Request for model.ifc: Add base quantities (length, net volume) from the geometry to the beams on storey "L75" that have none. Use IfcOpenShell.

First a look at what the model holds.

```python
import ifcopenshell
import ifcopenshell.util.element
import ifcopenshell.util.unit

model = ifcopenshell.open("model.ifc")
print(model.schema)
for unit_type in ("LENGTHUNIT", "AREAUNIT", "VOLUMEUNIT"):
    print(unit_type, ifcopenshell.util.unit.calculate_unit_scale(model, unit_type))
storey = next(s for s in model.by_type("IfcBuildingStorey") if s.Name == "L75")
beams = [e for e in ifcopenshell.util.element.get_decomposition(storey) if e.is_a("IfcBeam")]
for e in sorted(beams, key=lambda e: e.id()):
    print(e.id(), e.is_a(), e.Name, list(ifcopenshell.util.element.get_psets(e, qtos_only=True)), sep=" | ")
```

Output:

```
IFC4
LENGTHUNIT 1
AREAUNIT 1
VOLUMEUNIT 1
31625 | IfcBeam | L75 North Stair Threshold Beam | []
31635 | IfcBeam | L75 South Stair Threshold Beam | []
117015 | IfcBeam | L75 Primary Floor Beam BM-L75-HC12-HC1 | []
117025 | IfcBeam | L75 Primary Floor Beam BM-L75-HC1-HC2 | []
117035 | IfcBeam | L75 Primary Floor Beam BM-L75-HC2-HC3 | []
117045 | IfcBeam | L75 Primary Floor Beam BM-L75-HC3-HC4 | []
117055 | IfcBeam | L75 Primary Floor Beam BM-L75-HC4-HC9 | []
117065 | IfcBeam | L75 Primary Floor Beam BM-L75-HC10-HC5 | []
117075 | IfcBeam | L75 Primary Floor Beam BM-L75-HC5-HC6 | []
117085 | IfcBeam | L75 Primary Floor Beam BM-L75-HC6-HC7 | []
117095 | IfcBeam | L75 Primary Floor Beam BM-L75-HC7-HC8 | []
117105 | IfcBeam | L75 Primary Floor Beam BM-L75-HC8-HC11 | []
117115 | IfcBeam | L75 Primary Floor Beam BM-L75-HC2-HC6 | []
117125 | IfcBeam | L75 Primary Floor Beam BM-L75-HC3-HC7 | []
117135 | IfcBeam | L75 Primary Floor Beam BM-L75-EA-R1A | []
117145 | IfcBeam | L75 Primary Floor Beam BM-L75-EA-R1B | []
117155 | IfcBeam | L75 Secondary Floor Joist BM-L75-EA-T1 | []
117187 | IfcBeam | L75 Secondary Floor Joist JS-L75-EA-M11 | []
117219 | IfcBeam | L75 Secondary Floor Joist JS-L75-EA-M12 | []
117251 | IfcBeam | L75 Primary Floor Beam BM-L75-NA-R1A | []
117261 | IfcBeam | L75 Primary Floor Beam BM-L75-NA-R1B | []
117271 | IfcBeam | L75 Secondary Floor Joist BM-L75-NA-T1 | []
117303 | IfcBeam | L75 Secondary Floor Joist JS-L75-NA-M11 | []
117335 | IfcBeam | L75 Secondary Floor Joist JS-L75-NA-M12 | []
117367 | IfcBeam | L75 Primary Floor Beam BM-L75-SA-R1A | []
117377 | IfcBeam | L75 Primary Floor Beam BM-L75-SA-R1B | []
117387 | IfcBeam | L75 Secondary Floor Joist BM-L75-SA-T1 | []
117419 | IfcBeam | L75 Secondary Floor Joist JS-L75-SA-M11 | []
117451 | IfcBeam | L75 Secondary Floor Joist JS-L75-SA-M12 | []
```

```python
import ifcopenshell
import ifcopenshell.api.pset
import ifcopenshell.geom
import ifcopenshell.util.element
import ifcopenshell.util.shape
import ifcopenshell.util.unit

model = ifcopenshell.open("model.ifc")
unit_scale = ifcopenshell.util.unit.calculate_unit_scale(model)
volume_scale = ifcopenshell.util.unit.calculate_unit_scale(model, "VOLUMEUNIT")
settings = ifcopenshell.geom.settings()

storey = next(s for s in model.by_type("IfcBuildingStorey") if s.Name == "L75")
beams = [e for e in ifcopenshell.util.element.get_decomposition(storey) if e.is_a("IfcBeam")]

for e in sorted(beams, key=lambda e: e.id()):
    if ifcopenshell.util.element.get_psets(e, qtos_only=True, should_inherit=False):
        continue
    # Geometry comes back in metres, in the element's own axes.
    shape = ifcopenshell.geom.create_shape(settings, e)
    values = {
        "Length": ifcopenshell.util.shape.get_max_xyz(shape.geometry) / unit_scale,
        "NetVolume": ifcopenshell.util.shape.get_volume(shape.geometry) / volume_scale,
    }
    qto = ifcopenshell.api.pset.add_qto(model, product=e, name="Qto_BeamBaseQuantities")
    ifcopenshell.api.pset.edit_qto(model, qto=qto, properties=values)
    print(e.id(), {k: round(v, 3) for k, v in values.items()})

model.write("model_rev.ifc")
```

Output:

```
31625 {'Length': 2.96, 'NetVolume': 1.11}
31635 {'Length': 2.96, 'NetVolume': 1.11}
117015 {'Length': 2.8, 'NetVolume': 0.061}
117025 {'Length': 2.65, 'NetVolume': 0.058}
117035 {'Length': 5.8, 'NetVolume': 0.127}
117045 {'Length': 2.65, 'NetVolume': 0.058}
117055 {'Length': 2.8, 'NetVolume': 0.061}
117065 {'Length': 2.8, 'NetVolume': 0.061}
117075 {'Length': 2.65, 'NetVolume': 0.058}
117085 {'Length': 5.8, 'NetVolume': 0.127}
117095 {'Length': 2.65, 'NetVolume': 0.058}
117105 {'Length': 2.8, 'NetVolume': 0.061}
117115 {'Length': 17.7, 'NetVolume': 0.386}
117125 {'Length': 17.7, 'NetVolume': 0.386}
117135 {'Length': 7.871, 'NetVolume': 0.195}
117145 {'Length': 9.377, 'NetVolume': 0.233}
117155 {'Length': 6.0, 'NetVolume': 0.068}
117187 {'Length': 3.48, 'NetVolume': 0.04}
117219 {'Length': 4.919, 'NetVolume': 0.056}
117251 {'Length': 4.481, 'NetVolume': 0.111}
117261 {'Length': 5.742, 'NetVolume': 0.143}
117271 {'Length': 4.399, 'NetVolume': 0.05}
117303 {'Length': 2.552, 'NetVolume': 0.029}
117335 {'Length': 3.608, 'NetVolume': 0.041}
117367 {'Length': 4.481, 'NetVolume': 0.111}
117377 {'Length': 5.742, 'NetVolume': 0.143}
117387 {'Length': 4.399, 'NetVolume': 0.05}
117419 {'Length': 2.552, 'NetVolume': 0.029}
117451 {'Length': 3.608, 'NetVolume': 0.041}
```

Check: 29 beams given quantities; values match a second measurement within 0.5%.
